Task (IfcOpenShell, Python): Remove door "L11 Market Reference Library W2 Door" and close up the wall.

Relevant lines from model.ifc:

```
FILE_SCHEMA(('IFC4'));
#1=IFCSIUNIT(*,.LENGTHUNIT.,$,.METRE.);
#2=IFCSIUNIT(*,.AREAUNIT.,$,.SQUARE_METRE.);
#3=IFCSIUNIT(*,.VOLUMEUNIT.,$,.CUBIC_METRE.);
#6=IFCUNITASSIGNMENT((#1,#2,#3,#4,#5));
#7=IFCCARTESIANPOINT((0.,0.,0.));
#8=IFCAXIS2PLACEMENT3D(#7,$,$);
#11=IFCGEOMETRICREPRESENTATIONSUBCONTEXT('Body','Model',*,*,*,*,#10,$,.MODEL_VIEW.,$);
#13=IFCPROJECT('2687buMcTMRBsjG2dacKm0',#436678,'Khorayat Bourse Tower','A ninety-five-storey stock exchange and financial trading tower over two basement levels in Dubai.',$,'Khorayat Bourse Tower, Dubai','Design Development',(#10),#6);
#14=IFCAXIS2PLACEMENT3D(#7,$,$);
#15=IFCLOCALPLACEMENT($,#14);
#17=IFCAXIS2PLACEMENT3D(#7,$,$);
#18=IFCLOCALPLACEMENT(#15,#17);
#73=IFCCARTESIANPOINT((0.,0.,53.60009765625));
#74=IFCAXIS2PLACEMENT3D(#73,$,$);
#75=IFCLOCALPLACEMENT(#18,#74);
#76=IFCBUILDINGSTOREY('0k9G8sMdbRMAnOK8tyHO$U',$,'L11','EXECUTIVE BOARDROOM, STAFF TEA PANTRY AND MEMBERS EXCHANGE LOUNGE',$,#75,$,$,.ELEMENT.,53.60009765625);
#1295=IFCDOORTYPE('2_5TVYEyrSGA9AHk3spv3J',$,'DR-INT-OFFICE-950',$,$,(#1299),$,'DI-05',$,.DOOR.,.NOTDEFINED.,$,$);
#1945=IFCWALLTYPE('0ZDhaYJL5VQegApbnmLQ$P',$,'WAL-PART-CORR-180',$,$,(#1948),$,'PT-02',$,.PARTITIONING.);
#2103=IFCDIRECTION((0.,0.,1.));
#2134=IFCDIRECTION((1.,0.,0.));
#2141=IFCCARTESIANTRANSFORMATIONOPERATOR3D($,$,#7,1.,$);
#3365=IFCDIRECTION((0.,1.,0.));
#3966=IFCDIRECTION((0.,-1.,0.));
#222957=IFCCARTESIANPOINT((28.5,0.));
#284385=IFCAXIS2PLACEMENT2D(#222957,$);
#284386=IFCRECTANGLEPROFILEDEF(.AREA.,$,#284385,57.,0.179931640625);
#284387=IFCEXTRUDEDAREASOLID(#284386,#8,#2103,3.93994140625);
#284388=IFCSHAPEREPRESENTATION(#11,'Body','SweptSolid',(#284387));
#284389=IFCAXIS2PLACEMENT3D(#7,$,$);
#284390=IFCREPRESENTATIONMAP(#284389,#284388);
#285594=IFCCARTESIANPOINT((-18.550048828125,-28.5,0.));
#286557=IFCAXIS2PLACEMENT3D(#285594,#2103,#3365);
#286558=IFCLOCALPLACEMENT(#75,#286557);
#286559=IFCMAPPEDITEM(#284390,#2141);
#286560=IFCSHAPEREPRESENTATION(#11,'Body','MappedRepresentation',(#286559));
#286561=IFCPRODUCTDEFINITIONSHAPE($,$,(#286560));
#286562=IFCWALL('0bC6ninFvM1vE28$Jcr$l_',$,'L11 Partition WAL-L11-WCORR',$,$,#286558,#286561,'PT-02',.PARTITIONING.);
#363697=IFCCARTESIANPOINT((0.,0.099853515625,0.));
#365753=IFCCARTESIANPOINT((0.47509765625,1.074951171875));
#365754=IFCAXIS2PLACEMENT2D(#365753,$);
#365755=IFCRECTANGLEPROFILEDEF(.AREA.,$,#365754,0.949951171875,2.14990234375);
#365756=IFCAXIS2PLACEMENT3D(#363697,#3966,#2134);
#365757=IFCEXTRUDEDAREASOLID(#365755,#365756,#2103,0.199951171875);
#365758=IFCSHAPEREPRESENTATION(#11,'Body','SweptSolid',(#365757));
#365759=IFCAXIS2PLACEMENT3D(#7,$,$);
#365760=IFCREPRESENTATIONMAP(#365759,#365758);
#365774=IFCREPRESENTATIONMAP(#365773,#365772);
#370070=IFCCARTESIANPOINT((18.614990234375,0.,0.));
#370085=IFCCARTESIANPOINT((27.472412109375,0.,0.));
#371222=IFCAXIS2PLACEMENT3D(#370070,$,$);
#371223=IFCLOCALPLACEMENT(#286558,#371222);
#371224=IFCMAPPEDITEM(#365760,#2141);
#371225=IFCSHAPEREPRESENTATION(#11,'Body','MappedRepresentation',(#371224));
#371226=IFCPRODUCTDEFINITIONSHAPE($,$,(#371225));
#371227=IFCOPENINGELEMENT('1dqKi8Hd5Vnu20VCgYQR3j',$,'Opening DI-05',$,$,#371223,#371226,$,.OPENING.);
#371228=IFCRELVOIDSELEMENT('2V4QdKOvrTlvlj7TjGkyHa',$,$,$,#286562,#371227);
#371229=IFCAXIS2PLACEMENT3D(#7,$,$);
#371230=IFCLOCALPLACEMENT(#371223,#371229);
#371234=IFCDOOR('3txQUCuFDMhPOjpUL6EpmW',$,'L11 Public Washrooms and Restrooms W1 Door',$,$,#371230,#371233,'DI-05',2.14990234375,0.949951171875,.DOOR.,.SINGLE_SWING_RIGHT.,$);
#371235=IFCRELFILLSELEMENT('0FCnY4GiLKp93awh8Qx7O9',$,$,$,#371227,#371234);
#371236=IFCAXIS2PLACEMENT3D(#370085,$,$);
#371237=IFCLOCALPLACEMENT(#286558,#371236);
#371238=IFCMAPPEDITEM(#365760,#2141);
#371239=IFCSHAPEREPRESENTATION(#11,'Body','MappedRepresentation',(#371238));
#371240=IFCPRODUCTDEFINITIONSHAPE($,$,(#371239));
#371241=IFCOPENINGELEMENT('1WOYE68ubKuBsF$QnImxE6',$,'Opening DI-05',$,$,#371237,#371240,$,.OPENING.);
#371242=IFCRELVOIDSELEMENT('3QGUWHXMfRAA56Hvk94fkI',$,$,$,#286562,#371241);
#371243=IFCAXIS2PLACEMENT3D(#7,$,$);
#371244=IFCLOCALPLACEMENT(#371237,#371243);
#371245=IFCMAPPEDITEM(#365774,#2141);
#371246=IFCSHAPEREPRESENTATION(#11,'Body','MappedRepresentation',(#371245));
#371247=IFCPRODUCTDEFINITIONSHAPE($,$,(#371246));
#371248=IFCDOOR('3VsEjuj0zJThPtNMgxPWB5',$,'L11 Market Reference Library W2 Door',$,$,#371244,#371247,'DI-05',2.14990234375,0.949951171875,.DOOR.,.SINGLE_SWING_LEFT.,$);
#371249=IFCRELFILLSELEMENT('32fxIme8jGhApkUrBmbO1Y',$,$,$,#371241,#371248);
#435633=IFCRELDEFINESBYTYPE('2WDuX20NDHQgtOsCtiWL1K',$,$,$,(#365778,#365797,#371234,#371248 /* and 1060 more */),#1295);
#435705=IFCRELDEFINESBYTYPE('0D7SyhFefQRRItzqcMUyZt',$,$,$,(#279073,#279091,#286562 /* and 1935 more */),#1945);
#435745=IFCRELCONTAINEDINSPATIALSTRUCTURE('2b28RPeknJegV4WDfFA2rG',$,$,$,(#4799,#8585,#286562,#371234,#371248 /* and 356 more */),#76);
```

```python
import ifcopenshell
import ifcopenshell.api.feature
import ifcopenshell.api.root
import ifcopenshell.geom
import ifcopenshell.util.shape

model = ifcopenshell.open("model.ifc")
settings = ifcopenshell.geom.settings()


def volume(element):
    """Net volume in cubic metres, openings subtracted."""
    shape = ifcopenshell.geom.create_shape(settings, element)
    return ifcopenshell.util.shape.get_volume(shape.geometry)


door = model.by_id(371248)
opening = door.FillsVoids[0].RelatingOpeningElement
wall = opening.VoidsElements[0].RelatingBuildingElement
before = volume(wall)

ifcopenshell.api.root.remove_product(model, product=door)
ifcopenshell.api.feature.remove_feature(model, feature=opening)

after = volume(wall)

print(f"wall volume {before:.3f} -> {after:.3f} m3")

model.write("model_rev.ifc")
```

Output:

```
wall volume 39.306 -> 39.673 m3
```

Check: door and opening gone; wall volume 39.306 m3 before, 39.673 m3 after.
